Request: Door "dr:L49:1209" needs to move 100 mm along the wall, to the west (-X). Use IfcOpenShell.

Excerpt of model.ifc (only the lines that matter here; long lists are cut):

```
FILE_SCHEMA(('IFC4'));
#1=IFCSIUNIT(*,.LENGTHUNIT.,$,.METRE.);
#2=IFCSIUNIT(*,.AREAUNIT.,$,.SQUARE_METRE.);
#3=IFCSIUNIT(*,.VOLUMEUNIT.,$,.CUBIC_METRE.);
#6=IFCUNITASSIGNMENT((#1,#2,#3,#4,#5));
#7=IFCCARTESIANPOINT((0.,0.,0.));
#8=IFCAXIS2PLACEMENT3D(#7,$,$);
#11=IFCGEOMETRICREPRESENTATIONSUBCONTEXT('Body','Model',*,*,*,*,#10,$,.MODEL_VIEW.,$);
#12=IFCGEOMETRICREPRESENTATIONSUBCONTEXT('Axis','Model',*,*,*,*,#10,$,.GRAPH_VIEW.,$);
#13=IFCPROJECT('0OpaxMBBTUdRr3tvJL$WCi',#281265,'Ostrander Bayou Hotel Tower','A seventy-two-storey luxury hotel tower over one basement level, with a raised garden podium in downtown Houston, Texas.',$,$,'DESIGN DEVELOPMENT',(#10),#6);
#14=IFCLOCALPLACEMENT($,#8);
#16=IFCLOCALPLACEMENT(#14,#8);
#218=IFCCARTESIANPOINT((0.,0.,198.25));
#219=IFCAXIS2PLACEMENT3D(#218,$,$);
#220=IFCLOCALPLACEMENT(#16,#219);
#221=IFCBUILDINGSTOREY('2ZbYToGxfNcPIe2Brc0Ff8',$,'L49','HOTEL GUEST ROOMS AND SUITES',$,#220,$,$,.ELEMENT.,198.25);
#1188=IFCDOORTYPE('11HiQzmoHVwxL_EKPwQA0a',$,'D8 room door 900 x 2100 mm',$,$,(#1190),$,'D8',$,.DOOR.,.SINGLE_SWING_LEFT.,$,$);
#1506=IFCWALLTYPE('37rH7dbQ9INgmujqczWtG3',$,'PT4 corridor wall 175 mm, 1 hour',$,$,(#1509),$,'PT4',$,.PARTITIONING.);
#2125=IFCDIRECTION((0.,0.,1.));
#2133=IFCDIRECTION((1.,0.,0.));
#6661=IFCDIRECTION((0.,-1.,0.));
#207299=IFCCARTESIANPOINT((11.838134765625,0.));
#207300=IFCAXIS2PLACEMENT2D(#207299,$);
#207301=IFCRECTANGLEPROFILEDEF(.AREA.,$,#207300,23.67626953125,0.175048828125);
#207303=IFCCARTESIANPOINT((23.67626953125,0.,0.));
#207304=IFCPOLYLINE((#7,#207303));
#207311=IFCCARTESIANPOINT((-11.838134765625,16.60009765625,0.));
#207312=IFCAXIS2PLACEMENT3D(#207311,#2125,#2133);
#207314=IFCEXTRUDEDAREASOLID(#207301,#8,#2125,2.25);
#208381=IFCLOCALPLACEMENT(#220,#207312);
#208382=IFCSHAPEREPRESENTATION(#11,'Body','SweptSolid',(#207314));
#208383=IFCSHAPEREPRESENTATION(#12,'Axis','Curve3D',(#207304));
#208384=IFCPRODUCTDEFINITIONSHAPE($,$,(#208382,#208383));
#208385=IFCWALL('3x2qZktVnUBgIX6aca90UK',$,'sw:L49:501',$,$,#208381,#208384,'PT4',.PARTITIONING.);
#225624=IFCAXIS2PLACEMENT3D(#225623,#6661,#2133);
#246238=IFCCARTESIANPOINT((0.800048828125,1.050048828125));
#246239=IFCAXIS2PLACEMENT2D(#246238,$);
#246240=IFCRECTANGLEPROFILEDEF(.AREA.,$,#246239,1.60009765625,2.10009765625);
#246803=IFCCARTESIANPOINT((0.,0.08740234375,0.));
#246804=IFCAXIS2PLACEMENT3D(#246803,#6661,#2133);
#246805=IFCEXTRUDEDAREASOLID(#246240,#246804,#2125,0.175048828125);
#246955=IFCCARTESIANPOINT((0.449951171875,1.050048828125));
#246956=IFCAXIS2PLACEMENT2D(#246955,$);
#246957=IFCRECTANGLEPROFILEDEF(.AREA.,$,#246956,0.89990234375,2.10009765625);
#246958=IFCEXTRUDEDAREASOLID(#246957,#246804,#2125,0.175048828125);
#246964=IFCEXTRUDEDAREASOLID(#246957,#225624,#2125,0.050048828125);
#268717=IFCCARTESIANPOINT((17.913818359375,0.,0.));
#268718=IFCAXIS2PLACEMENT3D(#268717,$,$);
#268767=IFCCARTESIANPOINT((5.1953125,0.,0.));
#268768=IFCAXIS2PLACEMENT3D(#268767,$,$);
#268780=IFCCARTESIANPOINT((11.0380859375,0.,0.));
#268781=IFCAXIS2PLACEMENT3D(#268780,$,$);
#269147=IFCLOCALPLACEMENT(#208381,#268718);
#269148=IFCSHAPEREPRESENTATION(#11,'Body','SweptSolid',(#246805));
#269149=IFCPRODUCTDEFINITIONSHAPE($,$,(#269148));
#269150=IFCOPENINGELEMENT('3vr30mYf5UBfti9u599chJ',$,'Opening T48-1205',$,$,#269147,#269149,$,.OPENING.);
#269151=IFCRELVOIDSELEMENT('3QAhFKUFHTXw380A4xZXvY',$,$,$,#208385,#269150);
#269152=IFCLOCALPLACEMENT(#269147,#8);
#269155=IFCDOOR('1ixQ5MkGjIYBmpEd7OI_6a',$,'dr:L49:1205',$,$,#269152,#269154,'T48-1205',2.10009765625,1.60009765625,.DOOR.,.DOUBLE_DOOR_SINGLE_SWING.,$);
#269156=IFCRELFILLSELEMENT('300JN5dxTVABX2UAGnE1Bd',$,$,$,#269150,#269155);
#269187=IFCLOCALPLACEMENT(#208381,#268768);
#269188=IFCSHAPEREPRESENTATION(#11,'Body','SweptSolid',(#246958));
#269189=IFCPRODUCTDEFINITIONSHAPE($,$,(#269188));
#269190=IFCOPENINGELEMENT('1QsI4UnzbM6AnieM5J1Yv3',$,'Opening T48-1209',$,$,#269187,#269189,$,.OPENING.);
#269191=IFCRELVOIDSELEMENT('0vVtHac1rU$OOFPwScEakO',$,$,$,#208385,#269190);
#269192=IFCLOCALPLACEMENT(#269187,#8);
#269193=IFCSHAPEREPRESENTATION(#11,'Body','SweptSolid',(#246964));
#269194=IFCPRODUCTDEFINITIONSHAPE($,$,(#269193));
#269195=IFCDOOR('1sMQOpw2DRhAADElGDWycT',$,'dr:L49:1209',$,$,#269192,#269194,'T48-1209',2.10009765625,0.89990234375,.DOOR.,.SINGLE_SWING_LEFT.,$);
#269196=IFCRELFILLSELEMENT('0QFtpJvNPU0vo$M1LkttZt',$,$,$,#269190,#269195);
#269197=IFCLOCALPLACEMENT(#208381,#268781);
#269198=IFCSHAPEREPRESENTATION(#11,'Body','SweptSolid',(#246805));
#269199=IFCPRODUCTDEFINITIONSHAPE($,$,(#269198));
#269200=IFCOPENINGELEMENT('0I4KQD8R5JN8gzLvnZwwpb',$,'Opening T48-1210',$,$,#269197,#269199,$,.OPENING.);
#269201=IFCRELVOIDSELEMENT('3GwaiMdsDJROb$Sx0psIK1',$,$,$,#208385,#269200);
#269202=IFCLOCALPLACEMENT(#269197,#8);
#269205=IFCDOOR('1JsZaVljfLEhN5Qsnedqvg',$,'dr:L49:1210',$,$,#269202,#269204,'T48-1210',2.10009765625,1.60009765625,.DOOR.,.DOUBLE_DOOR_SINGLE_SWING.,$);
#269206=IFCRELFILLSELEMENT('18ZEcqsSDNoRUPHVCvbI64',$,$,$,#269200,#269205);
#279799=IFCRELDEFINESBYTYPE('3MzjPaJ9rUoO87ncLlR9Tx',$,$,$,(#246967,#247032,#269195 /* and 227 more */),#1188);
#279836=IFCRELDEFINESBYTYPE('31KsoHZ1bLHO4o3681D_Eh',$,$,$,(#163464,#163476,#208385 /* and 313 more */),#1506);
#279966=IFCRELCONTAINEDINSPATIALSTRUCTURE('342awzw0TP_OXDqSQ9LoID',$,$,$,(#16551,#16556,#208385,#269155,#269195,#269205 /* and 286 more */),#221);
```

```python
import ifcopenshell
import ifcopenshell.api.geometry
import ifcopenshell.util.placement
import ifcopenshell.util.unit

model = ifcopenshell.open("model.ifc")
unit_scale = ifcopenshell.util.unit.calculate_unit_scale(model)

door = model.by_id(269195)
opening = door.FillsVoids[0].RelatingOpeningElement
wall = opening.VoidsElements[0].RelatingBuildingElement

wall_matrix = ifcopenshell.util.placement.get_local_placement(wall.ObjectPlacement)
shift = wall_matrix[:3, 0] * -0.1 / unit_scale
before = ifcopenshell.util.placement.get_local_placement(door.ObjectPlacement)[:3, 3].copy()

# The door is placed relative to its opening, so it follows when the opening moves.
matrix = ifcopenshell.util.placement.get_local_placement(opening.ObjectPlacement)
matrix[:3, 3] += shift
ifcopenshell.api.geometry.edit_object_placement(
    model, product=opening, matrix=matrix, is_si=False, should_transform_children=True
)

after = ifcopenshell.util.placement.get_local_placement(door.ObjectPlacement)[:3, 3]
print("door moved by", (after - before).round(3) + 0.0)

model.write("model_v2.ifc")
```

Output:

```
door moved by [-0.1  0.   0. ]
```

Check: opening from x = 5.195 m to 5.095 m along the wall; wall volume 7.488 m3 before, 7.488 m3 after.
